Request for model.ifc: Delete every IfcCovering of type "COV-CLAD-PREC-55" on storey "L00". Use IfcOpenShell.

First a look at what the model holds.

```python
import ifcopenshell
import ifcopenshell.util.element

model = ifcopenshell.open("model.ifc")
print(model.schema)
storey = next(s for s in model.by_type("IfcBuildingStorey") if s.Name == "L00")
coverings = [e for e in ifcopenshell.util.element.get_decomposition(storey) if e.is_a("IfcCovering")]
seen = {}
for e in coverings:
    element_type = ifcopenshell.util.element.get_type(e)
    name = element_type.Name if element_type not in (None, e) else None
    seen[name] = seen.get(name, 0) + 1
for name, count in sorted(seen.items(), key=str):
    print(count, "x", name)
```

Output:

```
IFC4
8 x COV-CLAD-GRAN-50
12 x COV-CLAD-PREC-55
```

```python
import ifcopenshell
import ifcopenshell.api.root
import ifcopenshell.util.element

model = ifcopenshell.open("model.ifc")

storey = next(s for s in model.by_type("IfcBuildingStorey") if s.Name == "L00")
coverings = [e for e in ifcopenshell.util.element.get_decomposition(storey) if e.is_a("IfcCovering")]
targets = [e for e in coverings if (t := ifcopenshell.util.element.get_type(e)) not in (None, e) and t.Name == "COV-CLAD-PREC-55"]

for e in targets:
    ifcopenshell.api.root.remove_product(model, product=e)
print(len(targets), "removed")

model.write("model-out.ifc")
```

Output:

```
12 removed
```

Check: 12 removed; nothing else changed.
